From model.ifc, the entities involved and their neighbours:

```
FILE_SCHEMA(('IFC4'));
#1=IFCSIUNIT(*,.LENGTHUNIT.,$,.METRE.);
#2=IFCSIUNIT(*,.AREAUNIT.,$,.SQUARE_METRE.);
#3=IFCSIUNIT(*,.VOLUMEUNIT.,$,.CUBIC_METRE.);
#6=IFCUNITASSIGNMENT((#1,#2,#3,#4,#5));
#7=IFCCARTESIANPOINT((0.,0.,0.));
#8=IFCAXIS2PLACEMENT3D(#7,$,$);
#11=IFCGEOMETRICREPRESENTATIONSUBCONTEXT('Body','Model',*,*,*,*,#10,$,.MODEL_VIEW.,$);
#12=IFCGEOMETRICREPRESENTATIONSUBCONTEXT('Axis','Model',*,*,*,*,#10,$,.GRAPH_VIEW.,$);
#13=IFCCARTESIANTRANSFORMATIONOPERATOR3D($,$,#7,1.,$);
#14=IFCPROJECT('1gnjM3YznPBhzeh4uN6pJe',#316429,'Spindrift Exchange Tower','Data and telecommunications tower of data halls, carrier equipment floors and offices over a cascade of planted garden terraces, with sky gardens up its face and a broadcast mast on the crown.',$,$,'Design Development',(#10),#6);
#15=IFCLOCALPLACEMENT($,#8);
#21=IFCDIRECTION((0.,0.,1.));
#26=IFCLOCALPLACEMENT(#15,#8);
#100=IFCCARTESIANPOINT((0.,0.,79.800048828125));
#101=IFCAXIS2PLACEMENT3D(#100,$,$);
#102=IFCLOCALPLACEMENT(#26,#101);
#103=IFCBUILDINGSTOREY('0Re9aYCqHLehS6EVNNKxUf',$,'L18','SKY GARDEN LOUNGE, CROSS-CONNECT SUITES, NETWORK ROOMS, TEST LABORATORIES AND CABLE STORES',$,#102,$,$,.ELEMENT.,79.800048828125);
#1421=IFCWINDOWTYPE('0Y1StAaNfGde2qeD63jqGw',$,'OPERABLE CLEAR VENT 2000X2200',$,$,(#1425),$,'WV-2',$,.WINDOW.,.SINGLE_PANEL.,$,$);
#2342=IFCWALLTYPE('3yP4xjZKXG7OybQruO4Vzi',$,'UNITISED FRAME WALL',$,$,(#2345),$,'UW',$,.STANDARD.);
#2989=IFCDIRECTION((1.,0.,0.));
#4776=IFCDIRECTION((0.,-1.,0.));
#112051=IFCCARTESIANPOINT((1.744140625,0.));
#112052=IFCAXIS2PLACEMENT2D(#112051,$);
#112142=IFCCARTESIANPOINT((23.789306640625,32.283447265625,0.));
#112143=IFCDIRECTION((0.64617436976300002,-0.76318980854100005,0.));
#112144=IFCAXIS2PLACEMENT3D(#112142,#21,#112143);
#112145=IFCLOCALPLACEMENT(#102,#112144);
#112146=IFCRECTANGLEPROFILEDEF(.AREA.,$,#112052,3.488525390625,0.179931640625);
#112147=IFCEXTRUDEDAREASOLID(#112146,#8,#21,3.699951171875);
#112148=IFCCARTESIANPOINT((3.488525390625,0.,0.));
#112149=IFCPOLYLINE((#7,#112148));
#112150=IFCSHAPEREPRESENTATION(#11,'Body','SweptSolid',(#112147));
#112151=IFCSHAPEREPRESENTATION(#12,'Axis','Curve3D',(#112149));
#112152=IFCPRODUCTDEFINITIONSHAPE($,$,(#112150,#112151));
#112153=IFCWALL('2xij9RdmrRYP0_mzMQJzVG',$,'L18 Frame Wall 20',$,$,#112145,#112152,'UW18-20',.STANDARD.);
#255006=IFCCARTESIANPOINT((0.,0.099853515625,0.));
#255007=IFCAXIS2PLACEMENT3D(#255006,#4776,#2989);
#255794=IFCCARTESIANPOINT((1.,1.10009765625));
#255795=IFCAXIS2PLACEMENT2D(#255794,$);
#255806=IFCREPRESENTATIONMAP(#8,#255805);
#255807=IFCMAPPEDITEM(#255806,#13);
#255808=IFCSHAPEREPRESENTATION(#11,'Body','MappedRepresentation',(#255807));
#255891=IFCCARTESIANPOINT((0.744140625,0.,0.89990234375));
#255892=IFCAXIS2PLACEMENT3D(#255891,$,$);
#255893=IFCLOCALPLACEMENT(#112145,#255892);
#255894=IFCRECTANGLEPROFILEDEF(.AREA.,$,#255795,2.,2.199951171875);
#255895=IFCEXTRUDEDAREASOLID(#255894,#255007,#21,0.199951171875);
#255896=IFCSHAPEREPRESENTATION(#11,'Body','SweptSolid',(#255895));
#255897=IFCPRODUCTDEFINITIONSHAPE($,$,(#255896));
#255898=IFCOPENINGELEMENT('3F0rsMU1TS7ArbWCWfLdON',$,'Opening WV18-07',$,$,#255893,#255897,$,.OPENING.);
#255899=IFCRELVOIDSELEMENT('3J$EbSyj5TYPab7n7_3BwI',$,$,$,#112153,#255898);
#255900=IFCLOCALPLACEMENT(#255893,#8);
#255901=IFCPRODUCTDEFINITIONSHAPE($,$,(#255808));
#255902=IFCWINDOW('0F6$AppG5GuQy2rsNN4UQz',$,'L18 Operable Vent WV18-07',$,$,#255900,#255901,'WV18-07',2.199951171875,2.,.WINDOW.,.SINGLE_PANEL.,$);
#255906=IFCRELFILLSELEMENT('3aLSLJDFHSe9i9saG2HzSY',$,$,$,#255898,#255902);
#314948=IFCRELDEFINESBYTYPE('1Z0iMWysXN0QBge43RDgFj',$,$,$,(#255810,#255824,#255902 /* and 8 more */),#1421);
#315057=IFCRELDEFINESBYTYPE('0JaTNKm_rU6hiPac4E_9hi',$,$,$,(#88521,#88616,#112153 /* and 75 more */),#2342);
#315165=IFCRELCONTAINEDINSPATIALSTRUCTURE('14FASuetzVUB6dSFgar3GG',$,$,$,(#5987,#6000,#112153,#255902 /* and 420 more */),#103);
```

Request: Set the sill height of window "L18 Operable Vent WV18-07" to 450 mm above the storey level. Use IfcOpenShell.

```python
import numpy as np
import ifcopenshell
import ifcopenshell.api.geometry
import ifcopenshell.geom
import ifcopenshell.util.element
import ifcopenshell.util.placement
import ifcopenshell.util.shape
import ifcopenshell.util.unit

model = ifcopenshell.open("model.ifc")
unit_scale = ifcopenshell.util.unit.calculate_unit_scale(model)

window = model.by_id(255902)
opening = window.FillsVoids[0].RelatingOpeningElement
storey = ifcopenshell.util.element.get_container(window, ifc_class="IfcBuildingStorey")
level = ifcopenshell.util.placement.get_local_placement(storey.ObjectPlacement)[2, 3]

# The opening's origin need not be at the sill, so measure its lowest point.
shape = ifcopenshell.geom.create_shape(ifcopenshell.geom.settings(), opening)
bottom = ifcopenshell.util.shape.get_shape_bottom_elevation(shape, shape.geometry) / unit_scale
dz = level + 0.45 / unit_scale - bottom

shift = np.array([0.0, 0.0, dz])
# The window is placed relative to its opening, so it follows when the opening moves.
matrix = ifcopenshell.util.placement.get_local_placement(opening.ObjectPlacement)
matrix[:3, 3] += shift
ifcopenshell.api.geometry.edit_object_placement(
    model, product=opening, matrix=matrix, is_si=False, should_transform_children=True
)

print(f"moved by {dz * unit_scale:+.3f} m")

model.write("model_updated.ifc")
```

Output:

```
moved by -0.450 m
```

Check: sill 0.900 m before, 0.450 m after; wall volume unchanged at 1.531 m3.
